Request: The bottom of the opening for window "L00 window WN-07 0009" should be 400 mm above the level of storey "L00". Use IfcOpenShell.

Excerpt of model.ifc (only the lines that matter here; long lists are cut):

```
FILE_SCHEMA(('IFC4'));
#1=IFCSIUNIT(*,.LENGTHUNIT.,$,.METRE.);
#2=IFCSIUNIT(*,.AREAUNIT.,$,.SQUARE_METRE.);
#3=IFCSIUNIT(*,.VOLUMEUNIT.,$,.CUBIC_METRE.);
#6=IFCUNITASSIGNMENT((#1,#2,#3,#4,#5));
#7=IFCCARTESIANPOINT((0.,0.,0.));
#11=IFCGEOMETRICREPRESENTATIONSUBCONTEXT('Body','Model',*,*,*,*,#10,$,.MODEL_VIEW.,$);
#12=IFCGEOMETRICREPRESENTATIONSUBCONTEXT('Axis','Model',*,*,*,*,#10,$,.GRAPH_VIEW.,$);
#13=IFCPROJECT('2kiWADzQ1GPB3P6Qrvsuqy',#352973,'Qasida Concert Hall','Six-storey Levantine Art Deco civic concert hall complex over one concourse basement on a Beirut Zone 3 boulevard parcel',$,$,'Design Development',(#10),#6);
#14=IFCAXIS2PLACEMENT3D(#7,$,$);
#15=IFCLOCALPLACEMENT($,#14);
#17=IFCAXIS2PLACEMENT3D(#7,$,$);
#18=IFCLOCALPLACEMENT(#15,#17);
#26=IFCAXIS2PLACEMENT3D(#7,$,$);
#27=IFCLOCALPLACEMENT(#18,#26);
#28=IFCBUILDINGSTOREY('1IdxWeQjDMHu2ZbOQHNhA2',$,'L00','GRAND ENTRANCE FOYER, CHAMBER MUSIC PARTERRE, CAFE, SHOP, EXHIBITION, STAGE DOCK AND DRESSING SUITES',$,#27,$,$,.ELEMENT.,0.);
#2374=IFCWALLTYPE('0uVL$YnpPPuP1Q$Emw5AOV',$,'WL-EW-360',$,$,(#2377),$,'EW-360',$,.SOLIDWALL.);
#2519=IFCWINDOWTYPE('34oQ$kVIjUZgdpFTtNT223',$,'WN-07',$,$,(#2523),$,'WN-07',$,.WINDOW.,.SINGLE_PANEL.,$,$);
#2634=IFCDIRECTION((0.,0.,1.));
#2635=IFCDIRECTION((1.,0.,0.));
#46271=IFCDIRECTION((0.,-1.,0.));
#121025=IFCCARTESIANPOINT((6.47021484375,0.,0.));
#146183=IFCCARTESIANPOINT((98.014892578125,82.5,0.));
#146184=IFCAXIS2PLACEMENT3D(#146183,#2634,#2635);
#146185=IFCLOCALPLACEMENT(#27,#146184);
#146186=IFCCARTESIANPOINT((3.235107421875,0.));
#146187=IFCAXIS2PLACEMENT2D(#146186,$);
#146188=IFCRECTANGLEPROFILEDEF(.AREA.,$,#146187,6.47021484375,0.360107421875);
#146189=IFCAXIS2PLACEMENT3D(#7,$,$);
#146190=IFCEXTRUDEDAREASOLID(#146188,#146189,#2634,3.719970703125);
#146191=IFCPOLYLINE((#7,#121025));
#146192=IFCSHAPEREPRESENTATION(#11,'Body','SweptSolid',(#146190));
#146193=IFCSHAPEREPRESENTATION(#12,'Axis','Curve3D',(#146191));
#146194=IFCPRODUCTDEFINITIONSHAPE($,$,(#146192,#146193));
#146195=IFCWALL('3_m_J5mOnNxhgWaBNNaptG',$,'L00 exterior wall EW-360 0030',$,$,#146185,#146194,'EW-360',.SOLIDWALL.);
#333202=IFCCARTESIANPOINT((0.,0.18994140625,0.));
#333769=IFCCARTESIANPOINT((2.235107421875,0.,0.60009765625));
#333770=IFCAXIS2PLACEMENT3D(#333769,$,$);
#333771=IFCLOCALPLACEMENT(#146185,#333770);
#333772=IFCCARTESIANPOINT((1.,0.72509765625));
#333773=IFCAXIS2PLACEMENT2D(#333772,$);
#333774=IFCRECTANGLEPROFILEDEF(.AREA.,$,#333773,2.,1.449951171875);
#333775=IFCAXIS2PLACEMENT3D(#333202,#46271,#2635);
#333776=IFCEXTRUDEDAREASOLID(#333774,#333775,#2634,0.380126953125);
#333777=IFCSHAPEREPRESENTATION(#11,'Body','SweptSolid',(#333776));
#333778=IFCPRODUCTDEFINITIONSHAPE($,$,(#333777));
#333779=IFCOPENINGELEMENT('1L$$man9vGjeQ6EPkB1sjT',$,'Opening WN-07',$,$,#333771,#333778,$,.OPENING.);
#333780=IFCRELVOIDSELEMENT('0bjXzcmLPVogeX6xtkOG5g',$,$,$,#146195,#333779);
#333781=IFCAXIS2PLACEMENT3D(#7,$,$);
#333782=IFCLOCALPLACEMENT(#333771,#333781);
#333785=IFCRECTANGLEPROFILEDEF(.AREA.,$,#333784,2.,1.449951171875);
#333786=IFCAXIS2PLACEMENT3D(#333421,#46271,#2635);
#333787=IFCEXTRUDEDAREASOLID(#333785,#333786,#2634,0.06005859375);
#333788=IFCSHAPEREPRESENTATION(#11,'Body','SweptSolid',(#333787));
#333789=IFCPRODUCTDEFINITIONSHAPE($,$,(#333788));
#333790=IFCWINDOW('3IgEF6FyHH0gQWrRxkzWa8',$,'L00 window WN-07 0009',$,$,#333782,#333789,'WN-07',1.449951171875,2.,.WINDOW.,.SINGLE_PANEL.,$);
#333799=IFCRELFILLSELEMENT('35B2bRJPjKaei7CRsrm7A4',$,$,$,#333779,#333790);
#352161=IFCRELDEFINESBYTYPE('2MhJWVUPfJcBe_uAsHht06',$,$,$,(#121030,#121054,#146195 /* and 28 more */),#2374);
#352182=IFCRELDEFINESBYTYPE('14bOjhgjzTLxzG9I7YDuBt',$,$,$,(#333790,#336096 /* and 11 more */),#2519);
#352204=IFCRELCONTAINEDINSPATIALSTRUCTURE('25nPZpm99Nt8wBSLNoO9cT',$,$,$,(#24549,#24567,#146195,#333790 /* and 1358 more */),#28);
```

```python
import numpy as np
import ifcopenshell
import ifcopenshell.api.geometry
import ifcopenshell.geom
import ifcopenshell.util.element
import ifcopenshell.util.placement
import ifcopenshell.util.shape
import ifcopenshell.util.unit

model = ifcopenshell.open("model.ifc")
unit_scale = ifcopenshell.util.unit.calculate_unit_scale(model)

window = model.by_guid("3IgEF6FyHH0gQWrRxkzWa8")
opening = window.FillsVoids[0].RelatingOpeningElement
storey = ifcopenshell.util.element.get_container(window, ifc_class="IfcBuildingStorey")
level = ifcopenshell.util.placement.get_local_placement(storey.ObjectPlacement)[2, 3]

# The opening's origin need not be at the sill, so measure its lowest point.
shape = ifcopenshell.geom.create_shape(ifcopenshell.geom.settings(), opening)
bottom = ifcopenshell.util.shape.get_shape_bottom_elevation(shape, shape.geometry) / unit_scale
dz = level + 0.4 / unit_scale - bottom

shift = np.array([0.0, 0.0, dz])
# The window is placed relative to its opening, so it follows when the opening moves.
matrix = ifcopenshell.util.placement.get_local_placement(opening.ObjectPlacement)
matrix[:3, 3] += shift
ifcopenshell.api.geometry.edit_object_placement(
    model, product=opening, matrix=matrix, is_si=False, should_transform_children=True
)

print(f"moved by {dz * unit_scale:+.3f} m")

model.write("model_edited.ifc")
```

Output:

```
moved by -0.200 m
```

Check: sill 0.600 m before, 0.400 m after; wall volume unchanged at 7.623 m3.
